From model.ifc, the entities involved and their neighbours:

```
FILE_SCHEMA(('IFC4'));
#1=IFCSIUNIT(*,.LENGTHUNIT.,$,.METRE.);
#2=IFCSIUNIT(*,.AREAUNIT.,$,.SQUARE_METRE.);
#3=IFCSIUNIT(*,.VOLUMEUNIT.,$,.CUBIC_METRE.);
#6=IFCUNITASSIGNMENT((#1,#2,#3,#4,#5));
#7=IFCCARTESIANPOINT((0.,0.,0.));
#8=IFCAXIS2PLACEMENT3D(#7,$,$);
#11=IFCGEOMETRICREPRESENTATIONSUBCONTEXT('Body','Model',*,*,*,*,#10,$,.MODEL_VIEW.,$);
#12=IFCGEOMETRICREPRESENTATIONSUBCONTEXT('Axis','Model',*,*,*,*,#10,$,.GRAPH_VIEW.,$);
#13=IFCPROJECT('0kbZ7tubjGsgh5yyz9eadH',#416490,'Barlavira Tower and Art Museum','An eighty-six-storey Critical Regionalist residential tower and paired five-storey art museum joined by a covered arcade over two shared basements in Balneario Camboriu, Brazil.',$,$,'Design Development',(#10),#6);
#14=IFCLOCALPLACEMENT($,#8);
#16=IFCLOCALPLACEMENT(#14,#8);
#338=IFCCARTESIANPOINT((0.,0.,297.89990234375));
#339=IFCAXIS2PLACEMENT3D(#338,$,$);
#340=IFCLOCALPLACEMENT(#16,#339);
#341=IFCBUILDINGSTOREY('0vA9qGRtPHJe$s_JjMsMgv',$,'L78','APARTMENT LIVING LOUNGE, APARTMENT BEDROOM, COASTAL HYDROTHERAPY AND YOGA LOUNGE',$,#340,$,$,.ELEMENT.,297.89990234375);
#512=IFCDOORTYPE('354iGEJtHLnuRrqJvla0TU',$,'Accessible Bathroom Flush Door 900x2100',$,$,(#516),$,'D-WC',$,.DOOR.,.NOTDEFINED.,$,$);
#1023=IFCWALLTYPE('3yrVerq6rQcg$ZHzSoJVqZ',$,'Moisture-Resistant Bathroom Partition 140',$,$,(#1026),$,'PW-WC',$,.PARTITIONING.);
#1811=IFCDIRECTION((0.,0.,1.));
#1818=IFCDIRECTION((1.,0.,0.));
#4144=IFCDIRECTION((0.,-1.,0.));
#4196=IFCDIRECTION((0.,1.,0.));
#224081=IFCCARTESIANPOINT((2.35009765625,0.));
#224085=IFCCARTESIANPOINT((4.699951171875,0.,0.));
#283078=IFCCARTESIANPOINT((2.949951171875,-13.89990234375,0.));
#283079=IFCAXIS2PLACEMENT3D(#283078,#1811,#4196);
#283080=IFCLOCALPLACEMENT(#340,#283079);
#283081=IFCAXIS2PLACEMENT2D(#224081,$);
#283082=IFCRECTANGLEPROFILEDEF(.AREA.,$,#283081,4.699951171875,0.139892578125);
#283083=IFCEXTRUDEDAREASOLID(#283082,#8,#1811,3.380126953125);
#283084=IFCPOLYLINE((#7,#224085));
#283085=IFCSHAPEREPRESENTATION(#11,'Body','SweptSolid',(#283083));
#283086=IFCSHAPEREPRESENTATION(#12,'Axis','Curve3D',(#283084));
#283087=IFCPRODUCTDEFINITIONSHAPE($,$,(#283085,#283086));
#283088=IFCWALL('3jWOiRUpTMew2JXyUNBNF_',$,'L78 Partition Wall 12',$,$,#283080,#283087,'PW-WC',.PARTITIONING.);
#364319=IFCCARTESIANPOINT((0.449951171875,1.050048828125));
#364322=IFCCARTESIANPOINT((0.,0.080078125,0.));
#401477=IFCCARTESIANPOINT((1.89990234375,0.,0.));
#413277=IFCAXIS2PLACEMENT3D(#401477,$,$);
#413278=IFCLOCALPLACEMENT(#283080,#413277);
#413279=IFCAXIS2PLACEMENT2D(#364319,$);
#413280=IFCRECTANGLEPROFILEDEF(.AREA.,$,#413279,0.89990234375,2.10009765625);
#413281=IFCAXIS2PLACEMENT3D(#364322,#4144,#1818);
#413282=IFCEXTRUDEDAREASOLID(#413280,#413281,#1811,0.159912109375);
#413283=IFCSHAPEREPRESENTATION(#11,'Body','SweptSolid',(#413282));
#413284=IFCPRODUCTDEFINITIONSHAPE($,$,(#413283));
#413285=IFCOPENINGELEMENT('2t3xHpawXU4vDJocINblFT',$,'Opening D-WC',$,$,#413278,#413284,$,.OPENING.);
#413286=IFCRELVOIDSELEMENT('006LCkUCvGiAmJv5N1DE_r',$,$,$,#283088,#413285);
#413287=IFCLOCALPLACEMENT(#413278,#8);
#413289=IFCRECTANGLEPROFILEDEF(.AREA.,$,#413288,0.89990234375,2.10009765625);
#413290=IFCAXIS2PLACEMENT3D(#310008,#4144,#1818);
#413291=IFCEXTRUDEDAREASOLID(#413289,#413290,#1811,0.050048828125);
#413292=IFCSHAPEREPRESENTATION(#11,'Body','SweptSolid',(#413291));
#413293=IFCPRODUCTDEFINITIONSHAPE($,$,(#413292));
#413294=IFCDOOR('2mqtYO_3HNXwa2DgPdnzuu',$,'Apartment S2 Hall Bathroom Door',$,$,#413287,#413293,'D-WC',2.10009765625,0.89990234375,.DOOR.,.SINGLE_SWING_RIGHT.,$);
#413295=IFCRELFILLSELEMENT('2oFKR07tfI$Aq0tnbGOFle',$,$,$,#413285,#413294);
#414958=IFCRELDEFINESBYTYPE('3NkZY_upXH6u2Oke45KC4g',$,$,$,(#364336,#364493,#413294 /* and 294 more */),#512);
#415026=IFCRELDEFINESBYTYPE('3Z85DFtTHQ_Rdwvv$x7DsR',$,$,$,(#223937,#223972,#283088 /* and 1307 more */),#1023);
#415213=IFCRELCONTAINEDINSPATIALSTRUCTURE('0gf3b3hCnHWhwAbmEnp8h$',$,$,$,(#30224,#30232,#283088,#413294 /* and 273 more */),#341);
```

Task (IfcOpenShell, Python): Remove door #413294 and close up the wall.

```python
import ifcopenshell
import ifcopenshell.api.feature
import ifcopenshell.api.root
import ifcopenshell.geom
import ifcopenshell.util.shape

model = ifcopenshell.open("model.ifc")
settings = ifcopenshell.geom.settings()


def volume(element):
    """Net volume in cubic metres, openings subtracted."""
    shape = ifcopenshell.geom.create_shape(settings, element)
    return ifcopenshell.util.shape.get_volume(shape.geometry)


door = model.by_guid("2mqtYO_3HNXwa2DgPdnzuu")
opening = door.FillsVoids[0].RelatingOpeningElement
wall = opening.VoidsElements[0].RelatingBuildingElement
before = volume(wall)

ifcopenshell.api.root.remove_product(model, product=door)
ifcopenshell.api.feature.remove_feature(model, feature=opening)

after = volume(wall)

print(f"wall volume {before:.3f} -> {after:.3f} m3")

model.write("model_v2.ifc")
```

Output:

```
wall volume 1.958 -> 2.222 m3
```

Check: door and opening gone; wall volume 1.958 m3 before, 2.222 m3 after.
